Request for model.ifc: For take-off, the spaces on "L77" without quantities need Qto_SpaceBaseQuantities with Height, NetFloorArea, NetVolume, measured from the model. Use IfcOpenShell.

First a look at what the model holds.

```python
import ifcopenshell
import ifcopenshell.util.element
import ifcopenshell.util.unit

model = ifcopenshell.open("model.ifc")
print(model.schema)
for unit_type in ("LENGTHUNIT", "AREAUNIT", "VOLUMEUNIT"):
    print(unit_type, ifcopenshell.util.unit.calculate_unit_scale(model, unit_type))
storey = next(s for s in model.by_type("IfcBuildingStorey") if s.Name == "L77")
spaces = [e for e in ifcopenshell.util.element.get_decomposition(storey) if e.is_a("IfcSpace")]
for e in sorted(spaces, key=lambda e: e.id()):
    print(e.id(), e.is_a(), e.Name, list(ifcopenshell.util.element.get_psets(e, qtos_only=True)), sep=" | ")
```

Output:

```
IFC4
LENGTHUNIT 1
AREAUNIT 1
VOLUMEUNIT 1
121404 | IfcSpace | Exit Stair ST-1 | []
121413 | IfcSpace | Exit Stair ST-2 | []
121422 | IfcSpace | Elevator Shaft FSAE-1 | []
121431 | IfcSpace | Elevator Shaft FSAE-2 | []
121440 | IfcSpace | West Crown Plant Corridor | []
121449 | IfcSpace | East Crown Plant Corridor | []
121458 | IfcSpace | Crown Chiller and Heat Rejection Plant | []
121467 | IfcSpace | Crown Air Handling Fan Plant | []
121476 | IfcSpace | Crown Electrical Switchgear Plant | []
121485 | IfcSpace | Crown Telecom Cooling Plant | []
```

```python
import ifcopenshell
import ifcopenshell.api.pset
import ifcopenshell.geom
import ifcopenshell.util.element
import ifcopenshell.util.shape
import ifcopenshell.util.unit

model = ifcopenshell.open("model.ifc")
unit_scale = ifcopenshell.util.unit.calculate_unit_scale(model)
area_scale = ifcopenshell.util.unit.calculate_unit_scale(model, "AREAUNIT")
volume_scale = ifcopenshell.util.unit.calculate_unit_scale(model, "VOLUMEUNIT")
settings = ifcopenshell.geom.settings()

storey = next(s for s in model.by_type("IfcBuildingStorey") if s.Name == "L77")
spaces = [e for e in ifcopenshell.util.element.get_decomposition(storey) if e.is_a("IfcSpace")]

for e in sorted(spaces, key=lambda e: e.id()):
    if ifcopenshell.util.element.get_psets(e, qtos_only=True, should_inherit=False):
        continue
    # Geometry comes back in metres, in the element's own axes.
    shape = ifcopenshell.geom.create_shape(settings, e)
    values = {
        "Height": ifcopenshell.util.shape.get_z(shape.geometry) / unit_scale,
        "NetFloorArea": ifcopenshell.util.shape.get_footprint_area(shape.geometry) / area_scale,
        "NetVolume": ifcopenshell.util.shape.get_volume(shape.geometry) / volume_scale,
    }
    qto = ifcopenshell.api.pset.add_qto(model, product=e, name="Qto_SpaceBaseQuantities")
    ifcopenshell.api.pset.edit_qto(model, qto=qto, properties=values)
    print(e.id(), {k: round(v, 3) for k, v in values.items()})

model.write("model_edited.ifc")
```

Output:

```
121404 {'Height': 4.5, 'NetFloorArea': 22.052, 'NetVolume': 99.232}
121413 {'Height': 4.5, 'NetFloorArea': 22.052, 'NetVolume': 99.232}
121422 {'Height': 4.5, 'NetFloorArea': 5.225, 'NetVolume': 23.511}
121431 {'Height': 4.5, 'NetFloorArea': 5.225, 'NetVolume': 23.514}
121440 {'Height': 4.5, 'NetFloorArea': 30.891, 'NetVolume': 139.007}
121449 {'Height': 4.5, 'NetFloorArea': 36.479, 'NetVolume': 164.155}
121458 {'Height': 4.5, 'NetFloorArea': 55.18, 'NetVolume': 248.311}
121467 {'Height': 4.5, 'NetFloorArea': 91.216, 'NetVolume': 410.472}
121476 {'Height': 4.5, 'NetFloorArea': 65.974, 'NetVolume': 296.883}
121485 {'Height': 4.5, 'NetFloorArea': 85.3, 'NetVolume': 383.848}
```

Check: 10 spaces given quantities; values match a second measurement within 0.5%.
